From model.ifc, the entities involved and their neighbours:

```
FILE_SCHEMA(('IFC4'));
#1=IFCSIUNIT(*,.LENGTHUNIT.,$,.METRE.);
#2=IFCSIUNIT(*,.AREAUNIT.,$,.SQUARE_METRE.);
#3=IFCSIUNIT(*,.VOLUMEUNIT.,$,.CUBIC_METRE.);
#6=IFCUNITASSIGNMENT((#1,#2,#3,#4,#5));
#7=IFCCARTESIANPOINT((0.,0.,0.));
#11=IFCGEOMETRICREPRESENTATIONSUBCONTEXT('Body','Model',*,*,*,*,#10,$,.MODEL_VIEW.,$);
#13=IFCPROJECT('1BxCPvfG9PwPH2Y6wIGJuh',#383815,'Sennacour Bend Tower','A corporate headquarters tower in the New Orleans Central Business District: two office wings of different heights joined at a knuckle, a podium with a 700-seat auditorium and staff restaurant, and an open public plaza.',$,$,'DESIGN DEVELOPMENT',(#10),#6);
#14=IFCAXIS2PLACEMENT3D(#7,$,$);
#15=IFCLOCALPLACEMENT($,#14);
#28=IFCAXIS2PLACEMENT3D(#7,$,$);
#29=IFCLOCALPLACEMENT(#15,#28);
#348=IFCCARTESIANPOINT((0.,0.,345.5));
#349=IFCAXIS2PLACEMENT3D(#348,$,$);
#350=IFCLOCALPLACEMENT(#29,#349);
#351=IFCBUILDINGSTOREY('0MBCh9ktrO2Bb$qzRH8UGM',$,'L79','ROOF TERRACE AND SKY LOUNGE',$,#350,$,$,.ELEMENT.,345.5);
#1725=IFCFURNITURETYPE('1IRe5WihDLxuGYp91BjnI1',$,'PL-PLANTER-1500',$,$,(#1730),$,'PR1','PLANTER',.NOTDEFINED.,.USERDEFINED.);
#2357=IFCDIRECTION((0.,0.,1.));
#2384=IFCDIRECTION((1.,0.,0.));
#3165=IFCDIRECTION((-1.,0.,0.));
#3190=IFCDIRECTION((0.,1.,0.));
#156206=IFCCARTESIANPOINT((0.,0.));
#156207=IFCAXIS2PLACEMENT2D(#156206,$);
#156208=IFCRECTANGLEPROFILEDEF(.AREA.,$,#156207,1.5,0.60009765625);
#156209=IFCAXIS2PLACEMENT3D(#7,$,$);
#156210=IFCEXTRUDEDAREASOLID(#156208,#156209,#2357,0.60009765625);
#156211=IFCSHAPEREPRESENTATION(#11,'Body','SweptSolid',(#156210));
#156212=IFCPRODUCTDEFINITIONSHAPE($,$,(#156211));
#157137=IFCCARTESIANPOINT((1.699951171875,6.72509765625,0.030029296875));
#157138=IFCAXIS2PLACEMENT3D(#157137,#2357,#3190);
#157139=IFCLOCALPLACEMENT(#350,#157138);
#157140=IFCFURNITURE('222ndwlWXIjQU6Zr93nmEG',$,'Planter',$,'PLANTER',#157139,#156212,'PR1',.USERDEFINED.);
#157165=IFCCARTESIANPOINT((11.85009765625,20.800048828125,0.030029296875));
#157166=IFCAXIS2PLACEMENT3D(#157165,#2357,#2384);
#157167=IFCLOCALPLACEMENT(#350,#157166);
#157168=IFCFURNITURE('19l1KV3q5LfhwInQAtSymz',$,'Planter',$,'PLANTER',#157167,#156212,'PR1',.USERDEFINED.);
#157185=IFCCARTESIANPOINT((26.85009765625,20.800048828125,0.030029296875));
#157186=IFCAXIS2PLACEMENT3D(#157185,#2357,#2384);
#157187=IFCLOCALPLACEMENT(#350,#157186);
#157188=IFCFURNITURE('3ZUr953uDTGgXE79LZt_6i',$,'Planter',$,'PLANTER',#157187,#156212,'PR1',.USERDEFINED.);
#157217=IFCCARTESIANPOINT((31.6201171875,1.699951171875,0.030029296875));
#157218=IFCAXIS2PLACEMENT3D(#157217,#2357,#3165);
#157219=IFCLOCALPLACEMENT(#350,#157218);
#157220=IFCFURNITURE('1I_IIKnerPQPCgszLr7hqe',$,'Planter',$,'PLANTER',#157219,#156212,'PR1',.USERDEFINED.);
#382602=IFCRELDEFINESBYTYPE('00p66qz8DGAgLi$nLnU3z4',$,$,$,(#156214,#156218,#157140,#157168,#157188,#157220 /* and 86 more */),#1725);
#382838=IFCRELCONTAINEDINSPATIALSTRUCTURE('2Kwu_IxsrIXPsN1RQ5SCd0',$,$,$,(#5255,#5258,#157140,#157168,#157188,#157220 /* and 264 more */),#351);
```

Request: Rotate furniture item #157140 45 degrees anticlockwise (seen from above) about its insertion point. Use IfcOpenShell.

```python
import ifcopenshell
import ifcopenshell.api.geometry
import ifcopenshell.util.placement

model = ifcopenshell.open("model.ifc")

item = model.by_guid("222ndwlWXIjQU6Zr93nmEG")
matrix = ifcopenshell.util.placement.get_local_placement(item.ObjectPlacement)
matrix = matrix @ ifcopenshell.util.placement.rotation(45, "Z")
ifcopenshell.api.geometry.edit_object_placement(model, product=item, matrix=matrix, is_si=False)

print(ifcopenshell.util.placement.get_local_placement(item.ObjectPlacement).round(3) + 0.0)

model.write("model_rev.ifc")
```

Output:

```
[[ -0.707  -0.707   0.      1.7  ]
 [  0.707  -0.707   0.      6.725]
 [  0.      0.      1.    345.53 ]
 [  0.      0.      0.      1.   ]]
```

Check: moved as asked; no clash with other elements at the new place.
